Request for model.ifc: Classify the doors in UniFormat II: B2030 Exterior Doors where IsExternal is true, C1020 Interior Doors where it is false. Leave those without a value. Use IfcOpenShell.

First a look at what the model holds.

```python
import ifcopenshell
import ifcopenshell.util.element

model = ifcopenshell.open("model.ifc")
print(model.schema)
print("classifications:", [c.Name for c in model.by_type("IfcClassification")])
values = [ifcopenshell.util.element.get_pset(e, "Pset_DoorCommon", "IsExternal") for e in model.by_type("IfcDoor")]
for value in (True, False, None):
    print("IsExternal", value, values.count(value))
```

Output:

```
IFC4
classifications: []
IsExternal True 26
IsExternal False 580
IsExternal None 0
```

```python
import ifcopenshell
import ifcopenshell.api.classification
import ifcopenshell.util.element

model = ifcopenshell.open("model.ifc")

system = ifcopenshell.api.classification.add_classification(model, classification="UniFormat II")

doors = model.by_type("IfcDoor")
external = {e: ifcopenshell.util.element.get_pset(e, "Pset_DoorCommon", "IsExternal") for e in doors}
for flag, code, name in ((True, "B2030", "Exterior Doors"), (False, "C1020", "Interior Doors")):
    products = [e for e in doors if external[e] is flag]
    ifcopenshell.api.classification.add_reference(
        model, products=products, classification=system, identification=code, name=name
    )
    print(code, len(products))

model.write("model_rev.ifc")
```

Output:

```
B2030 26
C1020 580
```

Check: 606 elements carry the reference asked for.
